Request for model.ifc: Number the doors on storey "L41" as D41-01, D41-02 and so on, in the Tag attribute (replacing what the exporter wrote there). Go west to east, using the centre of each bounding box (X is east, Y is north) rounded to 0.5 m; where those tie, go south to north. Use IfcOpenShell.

First a look at what the model holds.

```python
import ifcopenshell
import ifcopenshell.util.element
import ifcopenshell.util.placement

model = ifcopenshell.open("model.ifc")
print(model.schema)
storey = next(s for s in model.by_type("IfcBuildingStorey") if s.Name == "L41")
doors = [e for e in ifcopenshell.util.element.get_decomposition(storey) if e.is_a("IfcDoor")]
for e in sorted(doors, key=lambda e: e.id()):
    origin = ifcopenshell.util.placement.get_local_placement(e.ObjectPlacement)[:3, 3]
    print(e.id(), e.Tag, e.Name, origin.round(2) + 0.0, sep=" | ")
```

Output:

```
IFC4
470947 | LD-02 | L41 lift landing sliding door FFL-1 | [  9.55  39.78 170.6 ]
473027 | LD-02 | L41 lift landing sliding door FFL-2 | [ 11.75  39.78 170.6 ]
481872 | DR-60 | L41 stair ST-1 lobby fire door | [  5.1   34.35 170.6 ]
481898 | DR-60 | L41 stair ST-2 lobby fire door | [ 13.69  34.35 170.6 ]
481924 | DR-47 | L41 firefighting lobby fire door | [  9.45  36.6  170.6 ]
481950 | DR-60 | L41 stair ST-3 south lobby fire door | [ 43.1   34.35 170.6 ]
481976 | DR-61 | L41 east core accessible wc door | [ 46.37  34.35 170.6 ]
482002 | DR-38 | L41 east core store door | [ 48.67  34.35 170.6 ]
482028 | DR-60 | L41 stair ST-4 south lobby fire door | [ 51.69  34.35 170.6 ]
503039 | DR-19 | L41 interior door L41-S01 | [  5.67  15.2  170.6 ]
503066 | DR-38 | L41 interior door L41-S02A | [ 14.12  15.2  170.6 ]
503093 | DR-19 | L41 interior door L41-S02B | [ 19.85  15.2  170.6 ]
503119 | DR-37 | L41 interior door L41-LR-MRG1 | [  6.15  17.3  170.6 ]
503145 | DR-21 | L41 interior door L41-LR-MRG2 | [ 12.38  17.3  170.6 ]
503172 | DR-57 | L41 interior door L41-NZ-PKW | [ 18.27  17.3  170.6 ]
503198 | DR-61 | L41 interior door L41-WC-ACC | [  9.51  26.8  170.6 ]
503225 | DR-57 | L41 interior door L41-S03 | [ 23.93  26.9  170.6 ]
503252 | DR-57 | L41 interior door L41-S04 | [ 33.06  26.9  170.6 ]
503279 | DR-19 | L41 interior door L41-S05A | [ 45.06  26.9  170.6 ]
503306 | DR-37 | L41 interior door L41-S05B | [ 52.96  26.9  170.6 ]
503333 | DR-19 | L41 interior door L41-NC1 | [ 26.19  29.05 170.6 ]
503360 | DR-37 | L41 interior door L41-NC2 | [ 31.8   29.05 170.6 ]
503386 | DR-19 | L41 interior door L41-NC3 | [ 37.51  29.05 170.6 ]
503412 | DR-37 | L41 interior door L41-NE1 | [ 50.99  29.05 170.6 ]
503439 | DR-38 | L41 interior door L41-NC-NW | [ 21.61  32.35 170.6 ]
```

```python
import ifcopenshell
import ifcopenshell.geom
import ifcopenshell.util.element
import ifcopenshell.util.shape

model = ifcopenshell.open("model.ifc")
settings = ifcopenshell.geom.settings()
settings.set("use-world-coords", True)


def centre(element):
    shape = ifcopenshell.geom.create_shape(settings, element)
    return ifcopenshell.util.shape.get_bbox_centroid(shape.geometry)


storey = next(s for s in model.by_type("IfcBuildingStorey") if s.Name == "L41")
doors = [e for e in ifcopenshell.util.element.get_decomposition(storey) if e.is_a("IfcDoor")]

# Insertion points can sit at a corner or the storey origin, so sort by the geometry (in metres).
centres = {e: centre(e) for e in doors}
doors.sort(key=lambda e: (round(centres[e][0] / 0.5), centres[e][1]))

for i, e in enumerate(doors, start=1):
    number = f"D41-{i:02d}"
    e.Tag = number
    print(e.id(), number)

model.write("model_edited.ifc")
```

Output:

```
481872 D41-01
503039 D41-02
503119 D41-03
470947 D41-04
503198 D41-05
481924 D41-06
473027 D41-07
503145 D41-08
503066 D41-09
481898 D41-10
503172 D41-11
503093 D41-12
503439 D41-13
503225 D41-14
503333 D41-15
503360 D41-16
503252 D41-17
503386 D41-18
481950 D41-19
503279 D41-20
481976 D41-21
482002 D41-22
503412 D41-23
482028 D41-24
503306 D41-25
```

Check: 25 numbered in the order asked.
